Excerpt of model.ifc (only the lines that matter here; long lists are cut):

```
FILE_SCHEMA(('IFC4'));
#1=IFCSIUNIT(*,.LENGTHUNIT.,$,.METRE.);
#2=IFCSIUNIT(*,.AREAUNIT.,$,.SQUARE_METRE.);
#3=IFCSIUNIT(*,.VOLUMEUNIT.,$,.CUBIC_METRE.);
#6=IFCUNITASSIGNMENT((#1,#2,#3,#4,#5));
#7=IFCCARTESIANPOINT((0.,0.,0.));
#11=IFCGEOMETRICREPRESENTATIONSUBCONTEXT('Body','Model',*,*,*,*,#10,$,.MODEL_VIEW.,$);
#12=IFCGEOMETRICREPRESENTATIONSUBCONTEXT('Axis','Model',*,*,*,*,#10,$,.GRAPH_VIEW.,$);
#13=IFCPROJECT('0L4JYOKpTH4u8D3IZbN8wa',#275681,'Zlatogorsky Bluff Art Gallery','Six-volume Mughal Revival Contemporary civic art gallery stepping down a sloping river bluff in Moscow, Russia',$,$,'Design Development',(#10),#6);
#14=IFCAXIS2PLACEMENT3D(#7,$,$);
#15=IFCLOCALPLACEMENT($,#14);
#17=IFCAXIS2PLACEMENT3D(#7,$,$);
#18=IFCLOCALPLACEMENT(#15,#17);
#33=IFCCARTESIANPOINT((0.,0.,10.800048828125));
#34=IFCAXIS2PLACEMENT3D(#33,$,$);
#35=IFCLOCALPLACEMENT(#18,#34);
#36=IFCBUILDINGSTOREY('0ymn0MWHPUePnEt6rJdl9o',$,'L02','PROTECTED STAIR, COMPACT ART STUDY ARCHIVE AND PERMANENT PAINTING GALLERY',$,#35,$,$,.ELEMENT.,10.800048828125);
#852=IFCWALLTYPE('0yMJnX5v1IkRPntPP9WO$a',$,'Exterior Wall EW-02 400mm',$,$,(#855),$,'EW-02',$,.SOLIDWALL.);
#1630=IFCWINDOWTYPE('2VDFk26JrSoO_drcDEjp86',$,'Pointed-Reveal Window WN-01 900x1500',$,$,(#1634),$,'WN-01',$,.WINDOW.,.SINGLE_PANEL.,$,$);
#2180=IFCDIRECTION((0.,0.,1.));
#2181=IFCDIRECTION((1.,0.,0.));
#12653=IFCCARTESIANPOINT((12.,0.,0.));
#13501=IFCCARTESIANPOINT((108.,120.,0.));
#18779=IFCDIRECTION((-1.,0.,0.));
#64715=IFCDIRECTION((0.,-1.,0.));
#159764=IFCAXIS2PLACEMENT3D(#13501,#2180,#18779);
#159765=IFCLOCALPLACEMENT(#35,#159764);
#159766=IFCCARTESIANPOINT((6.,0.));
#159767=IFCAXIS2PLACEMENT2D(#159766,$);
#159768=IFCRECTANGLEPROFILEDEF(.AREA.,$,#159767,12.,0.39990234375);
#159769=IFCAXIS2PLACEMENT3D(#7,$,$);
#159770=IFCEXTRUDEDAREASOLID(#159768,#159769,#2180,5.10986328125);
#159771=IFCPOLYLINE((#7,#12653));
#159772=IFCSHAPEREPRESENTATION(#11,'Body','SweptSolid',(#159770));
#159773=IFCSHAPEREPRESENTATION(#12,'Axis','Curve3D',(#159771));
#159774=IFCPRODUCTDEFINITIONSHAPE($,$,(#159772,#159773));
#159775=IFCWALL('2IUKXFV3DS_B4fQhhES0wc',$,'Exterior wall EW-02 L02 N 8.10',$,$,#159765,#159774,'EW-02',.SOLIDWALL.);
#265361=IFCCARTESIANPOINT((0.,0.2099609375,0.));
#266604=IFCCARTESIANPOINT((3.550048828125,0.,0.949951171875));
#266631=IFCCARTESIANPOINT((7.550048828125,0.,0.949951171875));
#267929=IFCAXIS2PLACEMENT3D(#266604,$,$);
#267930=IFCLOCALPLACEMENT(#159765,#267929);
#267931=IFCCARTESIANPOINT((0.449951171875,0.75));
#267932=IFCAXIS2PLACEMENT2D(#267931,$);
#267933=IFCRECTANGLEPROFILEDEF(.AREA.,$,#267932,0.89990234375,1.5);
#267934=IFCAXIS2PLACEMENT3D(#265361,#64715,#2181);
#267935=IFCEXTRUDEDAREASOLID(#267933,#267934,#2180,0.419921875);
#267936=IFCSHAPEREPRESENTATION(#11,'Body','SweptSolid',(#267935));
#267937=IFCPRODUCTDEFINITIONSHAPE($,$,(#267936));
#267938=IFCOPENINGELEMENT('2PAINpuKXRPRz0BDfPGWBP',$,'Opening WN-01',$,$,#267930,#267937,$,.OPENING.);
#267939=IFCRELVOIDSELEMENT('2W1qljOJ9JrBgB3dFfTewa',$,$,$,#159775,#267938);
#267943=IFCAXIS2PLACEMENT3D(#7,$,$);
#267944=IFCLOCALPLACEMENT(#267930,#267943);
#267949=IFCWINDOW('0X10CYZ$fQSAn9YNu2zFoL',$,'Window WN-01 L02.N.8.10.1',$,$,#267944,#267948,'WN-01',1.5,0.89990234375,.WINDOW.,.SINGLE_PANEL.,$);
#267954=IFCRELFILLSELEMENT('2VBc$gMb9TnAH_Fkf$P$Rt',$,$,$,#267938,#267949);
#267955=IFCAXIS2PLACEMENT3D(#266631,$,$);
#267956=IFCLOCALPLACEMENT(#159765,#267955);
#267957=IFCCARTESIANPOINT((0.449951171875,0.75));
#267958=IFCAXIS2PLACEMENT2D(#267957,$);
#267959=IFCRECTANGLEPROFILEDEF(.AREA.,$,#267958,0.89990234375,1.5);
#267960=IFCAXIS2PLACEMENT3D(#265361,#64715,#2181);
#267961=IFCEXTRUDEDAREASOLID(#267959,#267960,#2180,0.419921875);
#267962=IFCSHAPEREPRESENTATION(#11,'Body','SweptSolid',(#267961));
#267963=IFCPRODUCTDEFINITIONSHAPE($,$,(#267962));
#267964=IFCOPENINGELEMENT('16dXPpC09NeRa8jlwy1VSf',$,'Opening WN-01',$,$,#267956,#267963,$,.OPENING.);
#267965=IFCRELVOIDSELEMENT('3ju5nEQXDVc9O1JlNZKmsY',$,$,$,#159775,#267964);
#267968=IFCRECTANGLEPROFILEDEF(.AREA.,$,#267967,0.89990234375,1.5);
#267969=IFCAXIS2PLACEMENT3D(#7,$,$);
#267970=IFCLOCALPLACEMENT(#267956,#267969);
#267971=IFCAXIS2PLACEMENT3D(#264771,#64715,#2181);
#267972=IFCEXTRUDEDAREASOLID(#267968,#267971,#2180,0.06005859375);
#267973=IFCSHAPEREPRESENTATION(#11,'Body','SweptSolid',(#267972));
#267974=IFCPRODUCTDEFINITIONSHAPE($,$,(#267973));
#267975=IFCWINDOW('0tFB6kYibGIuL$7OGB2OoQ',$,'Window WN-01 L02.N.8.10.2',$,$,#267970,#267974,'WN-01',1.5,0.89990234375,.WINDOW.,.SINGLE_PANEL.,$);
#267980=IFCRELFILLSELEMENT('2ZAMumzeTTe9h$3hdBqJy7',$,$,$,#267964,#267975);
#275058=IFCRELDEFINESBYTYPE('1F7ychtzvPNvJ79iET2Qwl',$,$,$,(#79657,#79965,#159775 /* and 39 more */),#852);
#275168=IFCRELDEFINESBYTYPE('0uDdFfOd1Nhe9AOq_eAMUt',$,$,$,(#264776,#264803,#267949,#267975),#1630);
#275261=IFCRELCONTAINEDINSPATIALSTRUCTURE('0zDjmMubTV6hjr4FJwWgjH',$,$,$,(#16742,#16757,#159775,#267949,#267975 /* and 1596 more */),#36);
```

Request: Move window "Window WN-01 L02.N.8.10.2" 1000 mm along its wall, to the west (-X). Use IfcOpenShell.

```python
import ifcopenshell
import ifcopenshell.api.geometry
import ifcopenshell.util.placement
import ifcopenshell.util.unit

model = ifcopenshell.open("model.ifc")
unit_scale = ifcopenshell.util.unit.calculate_unit_scale(model)

window = model.by_guid("0tFB6kYibGIuL$7OGB2OoQ")
opening = window.FillsVoids[0].RelatingOpeningElement
wall = opening.VoidsElements[0].RelatingBuildingElement

wall_matrix = ifcopenshell.util.placement.get_local_placement(wall.ObjectPlacement)
shift = wall_matrix[:3, 0] * 1 / unit_scale
before = ifcopenshell.util.placement.get_local_placement(window.ObjectPlacement)[:3, 3].copy()

# The window is placed relative to its opening, so it follows when the opening moves.
matrix = ifcopenshell.util.placement.get_local_placement(opening.ObjectPlacement)
matrix[:3, 3] += shift
ifcopenshell.api.geometry.edit_object_placement(
    model, product=opening, matrix=matrix, is_si=False, should_transform_children=True
)

after = ifcopenshell.util.placement.get_local_placement(window.ObjectPlacement)[:3, 3]
print("window moved by", (after - before).round(3) + 0.0)

model.write("model_edited.ifc")
```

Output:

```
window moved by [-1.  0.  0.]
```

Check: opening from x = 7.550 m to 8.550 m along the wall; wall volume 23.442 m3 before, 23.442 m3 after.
